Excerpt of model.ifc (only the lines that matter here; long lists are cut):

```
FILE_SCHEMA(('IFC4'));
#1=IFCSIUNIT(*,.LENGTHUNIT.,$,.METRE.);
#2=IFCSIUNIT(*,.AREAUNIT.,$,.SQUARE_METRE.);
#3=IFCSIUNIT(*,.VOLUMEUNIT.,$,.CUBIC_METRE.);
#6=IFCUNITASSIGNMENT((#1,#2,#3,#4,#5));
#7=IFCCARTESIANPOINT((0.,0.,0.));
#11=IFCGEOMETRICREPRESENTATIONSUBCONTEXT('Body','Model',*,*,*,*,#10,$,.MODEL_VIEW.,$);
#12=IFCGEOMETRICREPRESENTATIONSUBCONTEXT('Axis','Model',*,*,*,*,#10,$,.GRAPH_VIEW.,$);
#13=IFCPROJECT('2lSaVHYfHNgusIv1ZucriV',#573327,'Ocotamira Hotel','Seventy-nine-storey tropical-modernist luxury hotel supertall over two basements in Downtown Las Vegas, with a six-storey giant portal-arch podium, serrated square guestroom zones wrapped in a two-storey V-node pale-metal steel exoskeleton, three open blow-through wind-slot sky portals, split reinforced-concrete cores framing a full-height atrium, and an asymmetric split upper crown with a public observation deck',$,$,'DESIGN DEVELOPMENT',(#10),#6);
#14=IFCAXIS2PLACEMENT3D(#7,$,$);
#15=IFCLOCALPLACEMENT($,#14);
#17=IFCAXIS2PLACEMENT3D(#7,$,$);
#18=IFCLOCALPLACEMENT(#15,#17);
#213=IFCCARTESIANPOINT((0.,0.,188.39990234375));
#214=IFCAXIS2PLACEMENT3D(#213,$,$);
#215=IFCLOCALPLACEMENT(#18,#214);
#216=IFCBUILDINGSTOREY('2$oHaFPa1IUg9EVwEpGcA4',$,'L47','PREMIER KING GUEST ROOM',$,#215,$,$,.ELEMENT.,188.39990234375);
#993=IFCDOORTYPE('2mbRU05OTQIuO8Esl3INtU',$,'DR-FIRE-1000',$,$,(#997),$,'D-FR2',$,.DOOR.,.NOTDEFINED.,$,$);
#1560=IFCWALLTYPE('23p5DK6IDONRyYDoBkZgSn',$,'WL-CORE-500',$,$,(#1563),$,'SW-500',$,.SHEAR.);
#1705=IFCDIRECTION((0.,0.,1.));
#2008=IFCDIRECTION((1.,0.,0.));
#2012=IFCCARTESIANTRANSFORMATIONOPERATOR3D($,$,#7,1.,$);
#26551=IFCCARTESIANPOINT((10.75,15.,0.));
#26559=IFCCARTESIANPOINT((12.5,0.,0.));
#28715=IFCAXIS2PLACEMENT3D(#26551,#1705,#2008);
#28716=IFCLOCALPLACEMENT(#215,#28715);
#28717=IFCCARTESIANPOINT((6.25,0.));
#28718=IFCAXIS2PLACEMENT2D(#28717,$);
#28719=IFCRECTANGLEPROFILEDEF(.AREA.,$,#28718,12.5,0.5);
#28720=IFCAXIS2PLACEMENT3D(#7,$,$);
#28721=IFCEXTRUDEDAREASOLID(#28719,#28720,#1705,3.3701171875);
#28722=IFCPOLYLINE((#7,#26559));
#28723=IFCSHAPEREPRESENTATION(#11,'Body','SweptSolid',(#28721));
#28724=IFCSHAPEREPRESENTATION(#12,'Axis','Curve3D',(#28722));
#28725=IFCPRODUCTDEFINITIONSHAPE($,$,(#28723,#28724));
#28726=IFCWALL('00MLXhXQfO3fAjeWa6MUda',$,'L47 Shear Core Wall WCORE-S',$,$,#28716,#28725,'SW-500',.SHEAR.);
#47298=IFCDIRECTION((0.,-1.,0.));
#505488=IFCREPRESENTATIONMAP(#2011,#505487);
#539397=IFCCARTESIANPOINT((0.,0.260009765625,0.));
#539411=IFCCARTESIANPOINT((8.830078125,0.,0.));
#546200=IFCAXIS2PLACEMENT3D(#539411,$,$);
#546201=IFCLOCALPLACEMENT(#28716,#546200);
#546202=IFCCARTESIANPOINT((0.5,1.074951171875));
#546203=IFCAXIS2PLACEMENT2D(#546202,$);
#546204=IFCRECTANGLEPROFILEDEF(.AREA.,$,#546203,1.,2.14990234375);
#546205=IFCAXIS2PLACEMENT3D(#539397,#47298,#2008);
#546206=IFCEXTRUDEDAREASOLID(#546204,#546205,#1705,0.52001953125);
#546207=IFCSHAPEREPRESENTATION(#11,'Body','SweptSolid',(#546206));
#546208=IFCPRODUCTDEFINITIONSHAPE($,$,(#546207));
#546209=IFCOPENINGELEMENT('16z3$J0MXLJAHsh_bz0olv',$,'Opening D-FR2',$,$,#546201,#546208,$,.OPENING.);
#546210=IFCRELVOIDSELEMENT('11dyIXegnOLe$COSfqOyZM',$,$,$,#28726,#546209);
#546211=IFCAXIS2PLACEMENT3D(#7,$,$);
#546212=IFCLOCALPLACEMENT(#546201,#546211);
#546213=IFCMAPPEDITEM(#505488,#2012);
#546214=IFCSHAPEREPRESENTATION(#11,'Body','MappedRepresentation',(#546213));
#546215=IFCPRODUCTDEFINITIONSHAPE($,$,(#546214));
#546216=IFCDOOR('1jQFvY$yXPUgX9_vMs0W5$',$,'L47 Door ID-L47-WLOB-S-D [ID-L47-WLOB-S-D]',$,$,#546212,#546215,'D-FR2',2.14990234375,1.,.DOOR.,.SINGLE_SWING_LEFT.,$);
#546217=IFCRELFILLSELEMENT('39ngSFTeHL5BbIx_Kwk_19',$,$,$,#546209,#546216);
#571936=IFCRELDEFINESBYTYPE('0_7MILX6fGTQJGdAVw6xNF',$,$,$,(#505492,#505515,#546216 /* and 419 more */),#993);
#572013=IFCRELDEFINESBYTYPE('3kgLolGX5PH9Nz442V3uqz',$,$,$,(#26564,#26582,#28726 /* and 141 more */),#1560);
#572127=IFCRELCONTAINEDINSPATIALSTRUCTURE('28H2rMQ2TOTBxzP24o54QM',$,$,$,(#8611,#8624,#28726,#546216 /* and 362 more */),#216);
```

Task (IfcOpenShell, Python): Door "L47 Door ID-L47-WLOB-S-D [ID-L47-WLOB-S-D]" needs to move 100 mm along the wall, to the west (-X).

```python
import ifcopenshell
import ifcopenshell.api.geometry
import ifcopenshell.util.placement

model = ifcopenshell.open("model.ifc")

door = model.by_id(546216)
opening = door.FillsVoids[0].RelatingOpeningElement
wall = opening.VoidsElements[0].RelatingBuildingElement

wall_matrix = ifcopenshell.util.placement.get_local_placement(wall.ObjectPlacement)
shift = wall_matrix[:3, 0] * -0.1
before = ifcopenshell.util.placement.get_local_placement(door.ObjectPlacement)[:3, 3].copy()

# The door is placed relative to its opening, so it follows when the opening moves.
matrix = ifcopenshell.util.placement.get_local_placement(opening.ObjectPlacement)
matrix[:3, 3] += shift
ifcopenshell.api.geometry.edit_object_placement(
    model, product=opening, matrix=matrix, is_si=False, should_transform_children=True
)

after = ifcopenshell.util.placement.get_local_placement(door.ObjectPlacement)[:3, 3]
print("door moved by", (after - before).round(3) + 0.0)

model.write("model_v2.ifc")
```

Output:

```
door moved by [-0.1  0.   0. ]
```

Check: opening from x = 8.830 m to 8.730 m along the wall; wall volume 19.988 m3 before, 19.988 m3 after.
